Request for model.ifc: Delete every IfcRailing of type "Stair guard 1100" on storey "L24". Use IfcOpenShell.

First a look at what the model holds.

```python
import ifcopenshell
import ifcopenshell.util.element

model = ifcopenshell.open("model.ifc")
print(model.schema)
storey = next(s for s in model.by_type("IfcBuildingStorey") if s.Name == "L24")
railings = [e for e in ifcopenshell.util.element.get_decomposition(storey) if e.is_a("IfcRailing")]
seen = {}
for e in railings:
    element_type = ifcopenshell.util.element.get_type(e)
    name = element_type.Name if element_type not in (None, e) else None
    seen[name] = seen.get(name, 0) + 1
for name, count in sorted(seen.items(), key=str):
    print(count, "x", name)
```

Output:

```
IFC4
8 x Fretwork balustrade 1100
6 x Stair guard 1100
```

```python
import ifcopenshell
import ifcopenshell.api.root
import ifcopenshell.util.element

model = ifcopenshell.open("model.ifc")

storey = next(s for s in model.by_type("IfcBuildingStorey") if s.Name == "L24")
railings = [e for e in ifcopenshell.util.element.get_decomposition(storey) if e.is_a("IfcRailing")]
targets = [e for e in railings if (t := ifcopenshell.util.element.get_type(e)) not in (None, e) and t.Name == "Stair guard 1100"]

for e in targets:
    ifcopenshell.api.root.remove_product(model, product=e)
print(len(targets), "removed")

model.write("model_rev.ifc")
```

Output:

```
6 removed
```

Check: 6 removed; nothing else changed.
